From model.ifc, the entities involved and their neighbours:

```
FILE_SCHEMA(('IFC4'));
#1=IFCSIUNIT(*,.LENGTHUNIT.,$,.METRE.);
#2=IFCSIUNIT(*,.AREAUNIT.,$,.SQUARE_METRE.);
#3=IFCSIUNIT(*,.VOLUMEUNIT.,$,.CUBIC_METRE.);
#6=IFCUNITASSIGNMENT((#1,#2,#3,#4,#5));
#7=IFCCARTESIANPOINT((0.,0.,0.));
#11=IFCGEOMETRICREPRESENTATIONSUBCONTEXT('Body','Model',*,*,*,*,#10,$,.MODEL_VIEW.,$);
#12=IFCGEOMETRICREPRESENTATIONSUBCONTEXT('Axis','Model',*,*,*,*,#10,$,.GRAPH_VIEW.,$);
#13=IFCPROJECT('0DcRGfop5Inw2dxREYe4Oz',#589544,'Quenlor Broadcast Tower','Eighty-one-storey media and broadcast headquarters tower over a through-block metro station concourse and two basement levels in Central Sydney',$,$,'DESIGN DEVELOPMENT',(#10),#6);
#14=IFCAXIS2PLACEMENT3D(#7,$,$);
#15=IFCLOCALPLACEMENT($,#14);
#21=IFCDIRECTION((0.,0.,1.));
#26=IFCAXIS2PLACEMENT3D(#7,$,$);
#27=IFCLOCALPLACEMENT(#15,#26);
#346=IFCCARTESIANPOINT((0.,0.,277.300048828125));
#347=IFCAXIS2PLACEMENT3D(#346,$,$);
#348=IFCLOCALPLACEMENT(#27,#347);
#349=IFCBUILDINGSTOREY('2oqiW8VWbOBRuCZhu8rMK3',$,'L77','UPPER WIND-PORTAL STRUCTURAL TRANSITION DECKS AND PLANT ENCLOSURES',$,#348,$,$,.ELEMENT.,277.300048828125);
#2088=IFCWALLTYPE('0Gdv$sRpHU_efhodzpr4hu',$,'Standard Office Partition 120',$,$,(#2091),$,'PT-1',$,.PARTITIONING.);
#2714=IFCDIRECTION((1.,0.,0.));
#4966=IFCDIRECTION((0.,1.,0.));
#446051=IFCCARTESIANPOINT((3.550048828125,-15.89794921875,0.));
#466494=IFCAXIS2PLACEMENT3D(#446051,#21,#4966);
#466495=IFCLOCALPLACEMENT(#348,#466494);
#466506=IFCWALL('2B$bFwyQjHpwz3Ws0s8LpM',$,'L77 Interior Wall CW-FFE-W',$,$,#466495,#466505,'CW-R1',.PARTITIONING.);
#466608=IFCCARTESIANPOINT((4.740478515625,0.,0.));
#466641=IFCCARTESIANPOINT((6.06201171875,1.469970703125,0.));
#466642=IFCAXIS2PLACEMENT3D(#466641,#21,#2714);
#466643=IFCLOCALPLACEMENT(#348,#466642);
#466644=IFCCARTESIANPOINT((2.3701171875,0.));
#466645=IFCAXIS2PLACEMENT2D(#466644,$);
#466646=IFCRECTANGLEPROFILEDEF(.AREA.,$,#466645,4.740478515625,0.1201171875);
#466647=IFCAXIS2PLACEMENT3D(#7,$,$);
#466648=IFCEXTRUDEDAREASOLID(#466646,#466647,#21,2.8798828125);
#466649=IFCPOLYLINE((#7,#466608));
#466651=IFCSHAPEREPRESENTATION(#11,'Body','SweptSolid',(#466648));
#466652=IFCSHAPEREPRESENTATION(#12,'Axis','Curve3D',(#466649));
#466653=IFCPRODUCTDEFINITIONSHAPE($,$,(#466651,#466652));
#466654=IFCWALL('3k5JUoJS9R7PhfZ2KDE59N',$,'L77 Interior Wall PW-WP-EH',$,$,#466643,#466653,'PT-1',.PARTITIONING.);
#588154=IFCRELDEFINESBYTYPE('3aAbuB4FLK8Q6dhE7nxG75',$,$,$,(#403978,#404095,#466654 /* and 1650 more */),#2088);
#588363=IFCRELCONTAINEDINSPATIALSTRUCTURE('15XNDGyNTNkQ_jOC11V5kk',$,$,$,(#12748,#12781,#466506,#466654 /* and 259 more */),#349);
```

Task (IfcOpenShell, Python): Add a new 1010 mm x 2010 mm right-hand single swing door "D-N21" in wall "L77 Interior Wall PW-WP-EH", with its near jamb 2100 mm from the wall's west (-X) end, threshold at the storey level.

```python
import numpy as np
import ifcopenshell
import ifcopenshell.api.feature
import ifcopenshell.api.geometry
import ifcopenshell.api.root
import ifcopenshell.api.spatial
import ifcopenshell.geom
import ifcopenshell.util.element
import ifcopenshell.util.placement
import ifcopenshell.util.representation
import ifcopenshell.util.shape
import ifcopenshell.util.unit

model = ifcopenshell.open("model.ifc")
unit_scale = ifcopenshell.util.unit.calculate_unit_scale(model)
settings = ifcopenshell.geom.settings()


def volume(element):
    """Net volume in cubic metres, openings subtracted."""
    shape = ifcopenshell.geom.create_shape(settings, element)
    return ifcopenshell.util.shape.get_volume(shape.geometry)


wall = model.by_guid("3k5JUoJS9R7PhfZ2KDE59N")
storey = ifcopenshell.util.element.get_container(wall, ifc_class="IfcBuildingStorey")
context = ifcopenshell.util.representation.get_context(model, "Model", "Body", "MODEL_VIEW")
before = volume(wall)

width, height, from_end, sill = 1.01, 2.01, 2.1, 0.0  # metres

# The wall runs along its own X axis, and the end named is its -X end.
wall_shape = ifcopenshell.geom.create_shape(settings, wall)
x, y, z = ifcopenshell.util.shape.get_vertices(wall_shape.geometry).T
start = x.min() + from_end
face, thickness = float(y.min()), float(y.max() - y.min())
wall_matrix = ifcopenshell.util.placement.get_local_placement(wall.ObjectPlacement)
level = ifcopenshell.util.placement.get_local_placement(storey.ObjectPlacement)[2, 3]


def in_wall(x, y):
    """Placement at x, y metres in the wall's axes, at sill height."""
    matrix = wall_matrix.copy()
    matrix[:, 3] = wall_matrix @ np.array([x / unit_scale, y / unit_scale, 0.0, 1.0])
    matrix[2, 3] = level + sill / unit_scale
    return matrix


# Opening: a box that overshoots both wall faces by 50 mm.
opening = ifcopenshell.api.root.create_entity(model, ifc_class="IfcOpeningElement", predefined_type="OPENING")
box = ifcopenshell.api.geometry.add_wall_representation(
    model, context=context, length=width, height=height, thickness=thickness + 0.1
)
ifcopenshell.api.geometry.assign_representation(model, product=opening, representation=box)
ifcopenshell.api.geometry.edit_object_placement(model, product=opening, matrix=in_wall(start, face - 0.05), is_si=False)
ifcopenshell.api.feature.add_feature(model, feature=opening, element=wall)

door = ifcopenshell.api.root.create_entity(model, ifc_class="IfcDoor", name="D-N21", predefined_type="DOOR")
door.OverallWidth, door.OverallHeight = width / unit_scale, height / unit_scale
door.OperationType = "SINGLE_SWING_RIGHT"
body = ifcopenshell.api.geometry.add_door_representation(
    model,
    context=context,
    overall_width=door.OverallWidth,
    overall_height=door.OverallHeight,
    operation_type="SINGLE_SWING_RIGHT",
    lining_properties={"LiningDepth": thickness / unit_scale, "ThresholdDepth": thickness / unit_scale},
)
ifcopenshell.api.geometry.assign_representation(model, product=door, representation=body)
ifcopenshell.api.spatial.assign_container(model, products=[door], relating_structure=storey)
ifcopenshell.api.feature.add_filling(model, opening=opening, element=door)

# The lining spans the wall, so the door starts at the wall face.
ifcopenshell.api.geometry.edit_object_placement(model, product=door, matrix=in_wall(start, face), is_si=False)

after = volume(wall)

print(f"wall volume {before:.3f} -> {after:.3f} m3")

model.write("model_updated.ifc")
```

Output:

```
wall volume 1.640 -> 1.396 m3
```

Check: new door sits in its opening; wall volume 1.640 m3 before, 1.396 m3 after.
